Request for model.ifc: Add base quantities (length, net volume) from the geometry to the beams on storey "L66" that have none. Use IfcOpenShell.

First a look at what the model holds.

```python
import ifcopenshell
import ifcopenshell.util.element
import ifcopenshell.util.unit

model = ifcopenshell.open("model.ifc")
print(model.schema)
for unit_type in ("LENGTHUNIT", "AREAUNIT", "VOLUMEUNIT"):
    print(unit_type, ifcopenshell.util.unit.calculate_unit_scale(model, unit_type))
storey = next(s for s in model.by_type("IfcBuildingStorey") if s.Name == "L66")
beams = [e for e in ifcopenshell.util.element.get_decomposition(storey) if e.is_a("IfcBeam")]
for e in sorted(beams, key=lambda e: e.id()):
    print(e.id(), e.is_a(), e.Name, list(ifcopenshell.util.element.get_psets(e, qtos_only=True)), sep=" | ")
```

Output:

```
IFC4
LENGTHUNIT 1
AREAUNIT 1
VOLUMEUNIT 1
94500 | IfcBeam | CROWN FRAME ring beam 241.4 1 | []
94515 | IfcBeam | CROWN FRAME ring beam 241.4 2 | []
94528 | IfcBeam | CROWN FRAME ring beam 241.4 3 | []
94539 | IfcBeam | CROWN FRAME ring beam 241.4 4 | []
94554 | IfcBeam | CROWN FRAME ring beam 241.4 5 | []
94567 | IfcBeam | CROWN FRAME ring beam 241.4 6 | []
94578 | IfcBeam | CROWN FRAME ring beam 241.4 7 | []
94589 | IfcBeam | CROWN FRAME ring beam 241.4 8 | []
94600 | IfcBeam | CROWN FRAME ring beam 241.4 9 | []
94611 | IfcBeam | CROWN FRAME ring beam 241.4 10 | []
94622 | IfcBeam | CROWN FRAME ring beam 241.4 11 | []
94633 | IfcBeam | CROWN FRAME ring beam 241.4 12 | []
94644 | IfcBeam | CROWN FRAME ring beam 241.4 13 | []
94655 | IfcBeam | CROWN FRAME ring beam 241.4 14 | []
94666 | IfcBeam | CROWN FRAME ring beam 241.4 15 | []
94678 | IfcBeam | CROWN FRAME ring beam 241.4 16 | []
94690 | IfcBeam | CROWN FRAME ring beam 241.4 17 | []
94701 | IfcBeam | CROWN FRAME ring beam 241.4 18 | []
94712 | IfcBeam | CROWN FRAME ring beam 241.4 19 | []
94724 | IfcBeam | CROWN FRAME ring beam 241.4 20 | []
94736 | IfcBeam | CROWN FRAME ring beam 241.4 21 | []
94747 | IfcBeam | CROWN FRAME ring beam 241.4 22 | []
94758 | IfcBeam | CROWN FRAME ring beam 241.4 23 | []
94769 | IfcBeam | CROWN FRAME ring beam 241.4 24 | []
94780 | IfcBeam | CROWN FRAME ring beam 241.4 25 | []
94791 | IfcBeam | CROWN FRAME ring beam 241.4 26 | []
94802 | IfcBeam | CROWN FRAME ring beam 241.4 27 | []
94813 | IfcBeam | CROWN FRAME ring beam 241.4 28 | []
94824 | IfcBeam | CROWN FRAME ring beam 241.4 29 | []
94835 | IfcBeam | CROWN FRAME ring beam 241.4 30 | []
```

```python
import ifcopenshell
import ifcopenshell.api.pset
import ifcopenshell.geom
import ifcopenshell.util.element
import ifcopenshell.util.shape
import ifcopenshell.util.unit

model = ifcopenshell.open("model.ifc")
unit_scale = ifcopenshell.util.unit.calculate_unit_scale(model)
volume_scale = ifcopenshell.util.unit.calculate_unit_scale(model, "VOLUMEUNIT")
settings = ifcopenshell.geom.settings()

storey = next(s for s in model.by_type("IfcBuildingStorey") if s.Name == "L66")
beams = [e for e in ifcopenshell.util.element.get_decomposition(storey) if e.is_a("IfcBeam")]

for e in sorted(beams, key=lambda e: e.id()):
    if ifcopenshell.util.element.get_psets(e, qtos_only=True, should_inherit=False):
        continue
    # Geometry comes back in metres, in the element's own axes.
    shape = ifcopenshell.geom.create_shape(settings, e)
    values = {
        "Length": ifcopenshell.util.shape.get_max_xyz(shape.geometry) / unit_scale,
        "NetVolume": ifcopenshell.util.shape.get_volume(shape.geometry) / volume_scale,
    }
    qto = ifcopenshell.api.pset.add_qto(model, product=e, name="Qto_BeamBaseQuantities")
    ifcopenshell.api.pset.edit_qto(model, qto=qto, properties=values)
    print(e.id(), {k: round(v, 3) for k, v in values.items()})

model.write("model-out.ifc")
```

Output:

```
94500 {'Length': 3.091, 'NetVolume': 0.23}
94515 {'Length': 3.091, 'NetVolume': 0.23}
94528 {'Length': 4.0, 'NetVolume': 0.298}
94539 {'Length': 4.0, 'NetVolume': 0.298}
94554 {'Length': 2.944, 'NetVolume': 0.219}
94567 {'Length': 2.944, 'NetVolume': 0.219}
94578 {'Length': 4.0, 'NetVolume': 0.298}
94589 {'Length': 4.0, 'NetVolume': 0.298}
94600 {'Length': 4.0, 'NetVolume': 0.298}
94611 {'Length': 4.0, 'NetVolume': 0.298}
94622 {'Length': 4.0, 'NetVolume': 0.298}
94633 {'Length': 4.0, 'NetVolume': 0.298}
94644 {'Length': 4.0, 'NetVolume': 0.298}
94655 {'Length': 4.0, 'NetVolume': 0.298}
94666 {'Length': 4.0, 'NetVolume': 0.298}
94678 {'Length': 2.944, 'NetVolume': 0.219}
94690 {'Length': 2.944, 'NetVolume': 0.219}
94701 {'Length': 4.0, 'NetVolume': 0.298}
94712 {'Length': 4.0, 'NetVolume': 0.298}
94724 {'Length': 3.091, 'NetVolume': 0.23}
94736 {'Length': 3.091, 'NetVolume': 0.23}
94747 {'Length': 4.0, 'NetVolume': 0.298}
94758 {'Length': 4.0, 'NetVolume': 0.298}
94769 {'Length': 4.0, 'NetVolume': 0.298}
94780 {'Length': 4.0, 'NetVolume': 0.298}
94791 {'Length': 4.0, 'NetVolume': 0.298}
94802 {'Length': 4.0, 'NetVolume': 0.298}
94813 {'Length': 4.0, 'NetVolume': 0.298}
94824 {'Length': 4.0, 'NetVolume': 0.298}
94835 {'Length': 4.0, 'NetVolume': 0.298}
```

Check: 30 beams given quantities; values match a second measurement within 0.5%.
